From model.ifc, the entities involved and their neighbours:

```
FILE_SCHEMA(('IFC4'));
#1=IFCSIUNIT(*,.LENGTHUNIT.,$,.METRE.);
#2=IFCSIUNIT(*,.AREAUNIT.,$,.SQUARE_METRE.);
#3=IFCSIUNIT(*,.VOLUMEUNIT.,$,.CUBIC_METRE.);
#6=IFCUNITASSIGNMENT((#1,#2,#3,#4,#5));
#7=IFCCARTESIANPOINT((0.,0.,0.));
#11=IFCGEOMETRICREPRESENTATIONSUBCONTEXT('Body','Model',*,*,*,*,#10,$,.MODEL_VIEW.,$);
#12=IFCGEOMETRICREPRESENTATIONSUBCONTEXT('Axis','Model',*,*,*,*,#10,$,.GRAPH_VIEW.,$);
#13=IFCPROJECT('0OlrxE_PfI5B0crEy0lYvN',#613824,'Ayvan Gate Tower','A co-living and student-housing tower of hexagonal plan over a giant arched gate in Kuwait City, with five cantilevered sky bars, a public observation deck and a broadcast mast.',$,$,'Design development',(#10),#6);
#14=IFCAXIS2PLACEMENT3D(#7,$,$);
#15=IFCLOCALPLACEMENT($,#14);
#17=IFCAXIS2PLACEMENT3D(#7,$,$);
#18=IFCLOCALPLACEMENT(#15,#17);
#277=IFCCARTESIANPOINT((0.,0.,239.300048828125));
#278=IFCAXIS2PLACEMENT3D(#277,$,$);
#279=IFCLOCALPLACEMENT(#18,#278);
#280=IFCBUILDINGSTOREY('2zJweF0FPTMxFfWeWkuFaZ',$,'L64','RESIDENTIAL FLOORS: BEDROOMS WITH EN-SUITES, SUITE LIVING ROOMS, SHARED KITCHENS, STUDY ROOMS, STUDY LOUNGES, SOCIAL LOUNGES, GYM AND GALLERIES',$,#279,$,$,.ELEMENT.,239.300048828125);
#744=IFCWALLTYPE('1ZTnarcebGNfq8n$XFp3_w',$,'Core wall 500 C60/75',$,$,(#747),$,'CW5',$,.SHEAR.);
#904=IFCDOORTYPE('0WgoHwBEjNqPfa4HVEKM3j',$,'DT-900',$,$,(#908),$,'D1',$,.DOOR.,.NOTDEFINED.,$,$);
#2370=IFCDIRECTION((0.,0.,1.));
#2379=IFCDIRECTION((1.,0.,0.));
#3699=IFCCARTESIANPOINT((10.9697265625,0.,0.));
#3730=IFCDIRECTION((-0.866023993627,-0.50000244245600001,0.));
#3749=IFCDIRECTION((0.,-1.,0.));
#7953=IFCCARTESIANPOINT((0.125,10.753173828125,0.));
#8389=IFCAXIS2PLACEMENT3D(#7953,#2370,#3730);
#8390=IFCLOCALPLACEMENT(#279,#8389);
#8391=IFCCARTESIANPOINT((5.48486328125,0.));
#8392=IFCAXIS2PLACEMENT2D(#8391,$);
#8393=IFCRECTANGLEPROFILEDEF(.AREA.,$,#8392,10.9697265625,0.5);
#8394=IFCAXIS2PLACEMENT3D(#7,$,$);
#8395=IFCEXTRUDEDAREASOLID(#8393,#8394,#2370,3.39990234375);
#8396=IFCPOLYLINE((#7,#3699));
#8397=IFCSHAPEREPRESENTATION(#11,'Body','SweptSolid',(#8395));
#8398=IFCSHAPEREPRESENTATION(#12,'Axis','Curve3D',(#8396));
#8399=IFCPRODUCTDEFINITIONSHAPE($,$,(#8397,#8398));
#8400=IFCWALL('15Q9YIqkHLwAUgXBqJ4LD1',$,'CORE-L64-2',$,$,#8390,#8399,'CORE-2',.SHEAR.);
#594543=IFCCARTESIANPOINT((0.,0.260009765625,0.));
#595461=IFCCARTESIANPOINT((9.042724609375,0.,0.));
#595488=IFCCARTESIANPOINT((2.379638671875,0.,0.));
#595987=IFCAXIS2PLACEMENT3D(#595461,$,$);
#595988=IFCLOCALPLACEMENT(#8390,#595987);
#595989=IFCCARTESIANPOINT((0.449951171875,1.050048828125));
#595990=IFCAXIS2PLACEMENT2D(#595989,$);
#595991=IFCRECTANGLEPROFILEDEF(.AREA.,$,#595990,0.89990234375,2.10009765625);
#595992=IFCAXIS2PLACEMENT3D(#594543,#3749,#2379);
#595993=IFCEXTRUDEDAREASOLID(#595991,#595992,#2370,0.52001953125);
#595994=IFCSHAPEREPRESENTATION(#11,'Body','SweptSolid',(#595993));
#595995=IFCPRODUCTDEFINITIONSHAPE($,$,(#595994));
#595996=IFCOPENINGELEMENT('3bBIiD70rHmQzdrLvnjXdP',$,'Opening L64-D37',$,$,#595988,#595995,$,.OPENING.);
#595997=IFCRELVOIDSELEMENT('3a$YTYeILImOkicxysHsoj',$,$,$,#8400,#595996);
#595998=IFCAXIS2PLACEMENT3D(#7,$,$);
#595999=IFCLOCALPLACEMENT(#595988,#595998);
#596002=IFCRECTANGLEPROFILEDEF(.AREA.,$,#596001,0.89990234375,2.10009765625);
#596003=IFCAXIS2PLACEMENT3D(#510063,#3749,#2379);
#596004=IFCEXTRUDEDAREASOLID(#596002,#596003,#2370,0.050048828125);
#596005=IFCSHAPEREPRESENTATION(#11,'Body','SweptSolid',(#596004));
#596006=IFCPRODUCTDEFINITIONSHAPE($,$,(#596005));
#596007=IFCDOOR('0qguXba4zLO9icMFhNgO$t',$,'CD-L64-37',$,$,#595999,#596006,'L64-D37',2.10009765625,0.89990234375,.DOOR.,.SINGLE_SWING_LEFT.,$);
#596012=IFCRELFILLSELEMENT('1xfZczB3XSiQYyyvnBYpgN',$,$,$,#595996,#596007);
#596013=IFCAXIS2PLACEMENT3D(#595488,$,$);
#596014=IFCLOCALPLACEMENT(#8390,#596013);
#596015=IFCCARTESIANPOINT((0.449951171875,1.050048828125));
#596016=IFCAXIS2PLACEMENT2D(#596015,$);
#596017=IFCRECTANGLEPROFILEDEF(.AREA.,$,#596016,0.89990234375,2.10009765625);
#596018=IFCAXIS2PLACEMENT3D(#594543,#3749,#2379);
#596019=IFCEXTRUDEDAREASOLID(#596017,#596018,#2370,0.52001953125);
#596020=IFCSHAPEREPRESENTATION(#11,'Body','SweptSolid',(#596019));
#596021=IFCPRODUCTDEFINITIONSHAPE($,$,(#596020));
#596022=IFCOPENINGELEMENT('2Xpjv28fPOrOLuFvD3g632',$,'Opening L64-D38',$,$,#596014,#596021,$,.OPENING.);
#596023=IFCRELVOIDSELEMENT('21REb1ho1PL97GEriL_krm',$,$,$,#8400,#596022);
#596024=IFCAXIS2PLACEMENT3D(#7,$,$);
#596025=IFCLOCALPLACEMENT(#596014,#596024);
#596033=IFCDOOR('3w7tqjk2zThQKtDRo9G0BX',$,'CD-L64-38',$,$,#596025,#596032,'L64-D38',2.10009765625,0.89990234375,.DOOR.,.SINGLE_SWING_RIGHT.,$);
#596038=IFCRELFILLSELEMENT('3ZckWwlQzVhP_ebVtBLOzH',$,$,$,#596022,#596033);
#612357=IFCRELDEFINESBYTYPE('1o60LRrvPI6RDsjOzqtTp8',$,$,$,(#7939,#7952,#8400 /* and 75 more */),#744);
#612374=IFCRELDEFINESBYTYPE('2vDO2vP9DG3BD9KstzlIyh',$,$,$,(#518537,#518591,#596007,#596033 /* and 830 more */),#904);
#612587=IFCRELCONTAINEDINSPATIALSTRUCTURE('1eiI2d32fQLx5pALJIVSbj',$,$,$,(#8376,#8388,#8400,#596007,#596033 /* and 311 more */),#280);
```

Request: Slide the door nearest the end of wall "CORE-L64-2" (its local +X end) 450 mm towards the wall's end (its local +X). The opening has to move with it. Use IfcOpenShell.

```python
import ifcopenshell
import ifcopenshell.api.geometry
import ifcopenshell.util.placement
import ifcopenshell.util.unit

model = ifcopenshell.open("model.ifc")
unit_scale = ifcopenshell.util.unit.calculate_unit_scale(model)

door = model.by_id(596007)
opening = door.FillsVoids[0].RelatingOpeningElement
wall = opening.VoidsElements[0].RelatingBuildingElement

wall_matrix = ifcopenshell.util.placement.get_local_placement(wall.ObjectPlacement)
shift = wall_matrix[:3, 0] * 0.45 / unit_scale
before = ifcopenshell.util.placement.get_local_placement(door.ObjectPlacement)[:3, 3].copy()

# The door is placed relative to its opening, so it follows when the opening moves.
matrix = ifcopenshell.util.placement.get_local_placement(opening.ObjectPlacement)
matrix[:3, 3] += shift
ifcopenshell.api.geometry.edit_object_placement(
    model, product=opening, matrix=matrix, is_si=False, should_transform_children=True
)

after = ifcopenshell.util.placement.get_local_placement(door.ObjectPlacement)[:3, 3]
print("door moved by", (after - before).round(3) + 0.0)

model.write("model_v2.ifc")
```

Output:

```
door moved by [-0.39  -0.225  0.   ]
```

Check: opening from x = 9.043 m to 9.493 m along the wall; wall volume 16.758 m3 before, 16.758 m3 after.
